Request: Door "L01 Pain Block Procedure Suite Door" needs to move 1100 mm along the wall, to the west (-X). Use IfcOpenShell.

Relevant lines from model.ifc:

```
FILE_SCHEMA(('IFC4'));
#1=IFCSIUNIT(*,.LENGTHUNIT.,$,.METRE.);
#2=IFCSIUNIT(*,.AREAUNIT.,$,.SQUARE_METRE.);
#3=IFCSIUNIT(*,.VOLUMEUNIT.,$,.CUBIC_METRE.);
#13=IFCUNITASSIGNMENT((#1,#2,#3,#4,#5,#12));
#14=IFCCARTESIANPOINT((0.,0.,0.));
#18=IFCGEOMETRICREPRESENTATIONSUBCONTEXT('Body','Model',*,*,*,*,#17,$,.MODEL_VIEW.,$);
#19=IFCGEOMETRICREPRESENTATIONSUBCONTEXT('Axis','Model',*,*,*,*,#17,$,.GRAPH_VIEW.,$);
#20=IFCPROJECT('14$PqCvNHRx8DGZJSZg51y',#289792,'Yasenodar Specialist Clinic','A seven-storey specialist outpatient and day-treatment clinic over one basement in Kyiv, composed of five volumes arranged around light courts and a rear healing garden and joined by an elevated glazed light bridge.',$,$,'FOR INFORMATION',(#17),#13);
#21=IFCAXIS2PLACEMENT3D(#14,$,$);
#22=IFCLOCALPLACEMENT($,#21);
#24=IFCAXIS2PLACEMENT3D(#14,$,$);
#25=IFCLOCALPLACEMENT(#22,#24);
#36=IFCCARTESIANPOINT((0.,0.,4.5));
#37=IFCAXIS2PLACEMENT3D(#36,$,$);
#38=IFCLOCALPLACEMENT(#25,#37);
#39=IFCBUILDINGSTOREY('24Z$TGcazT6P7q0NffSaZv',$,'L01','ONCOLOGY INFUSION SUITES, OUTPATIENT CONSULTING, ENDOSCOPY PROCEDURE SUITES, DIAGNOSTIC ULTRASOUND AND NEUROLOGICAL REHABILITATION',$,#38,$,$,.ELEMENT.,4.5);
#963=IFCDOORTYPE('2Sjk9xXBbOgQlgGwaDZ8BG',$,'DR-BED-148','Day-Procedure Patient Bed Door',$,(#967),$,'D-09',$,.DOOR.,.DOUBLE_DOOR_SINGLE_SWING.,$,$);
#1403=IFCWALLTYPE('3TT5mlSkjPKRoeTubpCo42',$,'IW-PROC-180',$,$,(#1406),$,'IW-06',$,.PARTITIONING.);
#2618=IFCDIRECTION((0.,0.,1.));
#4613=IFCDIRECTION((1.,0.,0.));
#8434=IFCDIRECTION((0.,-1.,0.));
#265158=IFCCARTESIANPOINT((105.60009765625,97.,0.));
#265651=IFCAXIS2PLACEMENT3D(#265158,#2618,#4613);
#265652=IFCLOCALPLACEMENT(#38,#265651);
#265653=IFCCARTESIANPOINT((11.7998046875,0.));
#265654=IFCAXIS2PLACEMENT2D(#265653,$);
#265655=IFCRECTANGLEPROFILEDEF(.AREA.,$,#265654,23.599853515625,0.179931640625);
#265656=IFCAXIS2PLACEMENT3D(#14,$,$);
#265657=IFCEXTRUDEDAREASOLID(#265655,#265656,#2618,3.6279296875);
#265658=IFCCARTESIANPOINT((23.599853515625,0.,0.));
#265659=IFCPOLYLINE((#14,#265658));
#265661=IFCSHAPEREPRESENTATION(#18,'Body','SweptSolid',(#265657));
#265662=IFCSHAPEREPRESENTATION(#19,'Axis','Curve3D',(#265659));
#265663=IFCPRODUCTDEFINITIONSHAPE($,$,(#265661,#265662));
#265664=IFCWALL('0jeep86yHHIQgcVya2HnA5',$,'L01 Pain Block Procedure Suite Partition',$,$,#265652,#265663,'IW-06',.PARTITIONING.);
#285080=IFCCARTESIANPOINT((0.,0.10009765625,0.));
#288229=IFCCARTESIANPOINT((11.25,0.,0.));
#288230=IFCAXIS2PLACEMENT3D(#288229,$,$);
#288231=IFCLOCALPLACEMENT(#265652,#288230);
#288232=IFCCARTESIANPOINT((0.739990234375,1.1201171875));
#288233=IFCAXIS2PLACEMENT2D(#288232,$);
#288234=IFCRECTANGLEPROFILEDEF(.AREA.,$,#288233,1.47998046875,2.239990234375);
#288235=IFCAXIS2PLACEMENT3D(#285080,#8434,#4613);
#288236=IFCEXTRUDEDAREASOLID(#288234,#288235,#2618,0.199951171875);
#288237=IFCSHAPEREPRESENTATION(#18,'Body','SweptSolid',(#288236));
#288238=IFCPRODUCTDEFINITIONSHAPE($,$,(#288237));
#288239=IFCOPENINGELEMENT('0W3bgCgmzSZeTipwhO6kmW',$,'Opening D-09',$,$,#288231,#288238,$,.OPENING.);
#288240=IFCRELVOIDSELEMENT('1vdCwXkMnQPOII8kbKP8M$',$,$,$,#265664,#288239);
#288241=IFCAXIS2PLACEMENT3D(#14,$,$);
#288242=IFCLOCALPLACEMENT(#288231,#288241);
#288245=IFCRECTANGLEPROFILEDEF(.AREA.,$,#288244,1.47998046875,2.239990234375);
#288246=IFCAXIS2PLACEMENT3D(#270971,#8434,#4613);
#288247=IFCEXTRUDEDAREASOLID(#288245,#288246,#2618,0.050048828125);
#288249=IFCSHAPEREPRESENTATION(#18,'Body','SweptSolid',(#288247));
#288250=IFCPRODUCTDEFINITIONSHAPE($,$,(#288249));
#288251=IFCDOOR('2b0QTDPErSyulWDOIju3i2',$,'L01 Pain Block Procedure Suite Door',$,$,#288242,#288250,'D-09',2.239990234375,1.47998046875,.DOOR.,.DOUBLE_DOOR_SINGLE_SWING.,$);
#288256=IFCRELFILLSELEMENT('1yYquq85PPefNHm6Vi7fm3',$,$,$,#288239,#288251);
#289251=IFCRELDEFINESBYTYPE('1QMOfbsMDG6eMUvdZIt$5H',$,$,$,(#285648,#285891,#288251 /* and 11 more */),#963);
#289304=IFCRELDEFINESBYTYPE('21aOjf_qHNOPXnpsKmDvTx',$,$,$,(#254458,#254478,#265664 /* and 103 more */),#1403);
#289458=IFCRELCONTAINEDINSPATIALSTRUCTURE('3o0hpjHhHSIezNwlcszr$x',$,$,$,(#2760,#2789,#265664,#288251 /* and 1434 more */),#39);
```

```python
import ifcopenshell
import ifcopenshell.api.geometry
import ifcopenshell.util.placement

model = ifcopenshell.open("model.ifc")

door = model.by_guid("2b0QTDPErSyulWDOIju3i2")
opening = door.FillsVoids[0].RelatingOpeningElement
wall = opening.VoidsElements[0].RelatingBuildingElement

wall_matrix = ifcopenshell.util.placement.get_local_placement(wall.ObjectPlacement)
shift = wall_matrix[:3, 0] * -1.1
before = ifcopenshell.util.placement.get_local_placement(door.ObjectPlacement)[:3, 3].copy()

# The door is placed relative to its opening, so it follows when the opening moves.
matrix = ifcopenshell.util.placement.get_local_placement(opening.ObjectPlacement)
matrix[:3, 3] += shift
ifcopenshell.api.geometry.edit_object_placement(
    model, product=opening, matrix=matrix, is_si=False, should_transform_children=True
)

after = ifcopenshell.util.placement.get_local_placement(door.ObjectPlacement)[:3, 3]
print("door moved by", (after - before).round(3) + 0.0)

model.write("model_v2.ifc")
```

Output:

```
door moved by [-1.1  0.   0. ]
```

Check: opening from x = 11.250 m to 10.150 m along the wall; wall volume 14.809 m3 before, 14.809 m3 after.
